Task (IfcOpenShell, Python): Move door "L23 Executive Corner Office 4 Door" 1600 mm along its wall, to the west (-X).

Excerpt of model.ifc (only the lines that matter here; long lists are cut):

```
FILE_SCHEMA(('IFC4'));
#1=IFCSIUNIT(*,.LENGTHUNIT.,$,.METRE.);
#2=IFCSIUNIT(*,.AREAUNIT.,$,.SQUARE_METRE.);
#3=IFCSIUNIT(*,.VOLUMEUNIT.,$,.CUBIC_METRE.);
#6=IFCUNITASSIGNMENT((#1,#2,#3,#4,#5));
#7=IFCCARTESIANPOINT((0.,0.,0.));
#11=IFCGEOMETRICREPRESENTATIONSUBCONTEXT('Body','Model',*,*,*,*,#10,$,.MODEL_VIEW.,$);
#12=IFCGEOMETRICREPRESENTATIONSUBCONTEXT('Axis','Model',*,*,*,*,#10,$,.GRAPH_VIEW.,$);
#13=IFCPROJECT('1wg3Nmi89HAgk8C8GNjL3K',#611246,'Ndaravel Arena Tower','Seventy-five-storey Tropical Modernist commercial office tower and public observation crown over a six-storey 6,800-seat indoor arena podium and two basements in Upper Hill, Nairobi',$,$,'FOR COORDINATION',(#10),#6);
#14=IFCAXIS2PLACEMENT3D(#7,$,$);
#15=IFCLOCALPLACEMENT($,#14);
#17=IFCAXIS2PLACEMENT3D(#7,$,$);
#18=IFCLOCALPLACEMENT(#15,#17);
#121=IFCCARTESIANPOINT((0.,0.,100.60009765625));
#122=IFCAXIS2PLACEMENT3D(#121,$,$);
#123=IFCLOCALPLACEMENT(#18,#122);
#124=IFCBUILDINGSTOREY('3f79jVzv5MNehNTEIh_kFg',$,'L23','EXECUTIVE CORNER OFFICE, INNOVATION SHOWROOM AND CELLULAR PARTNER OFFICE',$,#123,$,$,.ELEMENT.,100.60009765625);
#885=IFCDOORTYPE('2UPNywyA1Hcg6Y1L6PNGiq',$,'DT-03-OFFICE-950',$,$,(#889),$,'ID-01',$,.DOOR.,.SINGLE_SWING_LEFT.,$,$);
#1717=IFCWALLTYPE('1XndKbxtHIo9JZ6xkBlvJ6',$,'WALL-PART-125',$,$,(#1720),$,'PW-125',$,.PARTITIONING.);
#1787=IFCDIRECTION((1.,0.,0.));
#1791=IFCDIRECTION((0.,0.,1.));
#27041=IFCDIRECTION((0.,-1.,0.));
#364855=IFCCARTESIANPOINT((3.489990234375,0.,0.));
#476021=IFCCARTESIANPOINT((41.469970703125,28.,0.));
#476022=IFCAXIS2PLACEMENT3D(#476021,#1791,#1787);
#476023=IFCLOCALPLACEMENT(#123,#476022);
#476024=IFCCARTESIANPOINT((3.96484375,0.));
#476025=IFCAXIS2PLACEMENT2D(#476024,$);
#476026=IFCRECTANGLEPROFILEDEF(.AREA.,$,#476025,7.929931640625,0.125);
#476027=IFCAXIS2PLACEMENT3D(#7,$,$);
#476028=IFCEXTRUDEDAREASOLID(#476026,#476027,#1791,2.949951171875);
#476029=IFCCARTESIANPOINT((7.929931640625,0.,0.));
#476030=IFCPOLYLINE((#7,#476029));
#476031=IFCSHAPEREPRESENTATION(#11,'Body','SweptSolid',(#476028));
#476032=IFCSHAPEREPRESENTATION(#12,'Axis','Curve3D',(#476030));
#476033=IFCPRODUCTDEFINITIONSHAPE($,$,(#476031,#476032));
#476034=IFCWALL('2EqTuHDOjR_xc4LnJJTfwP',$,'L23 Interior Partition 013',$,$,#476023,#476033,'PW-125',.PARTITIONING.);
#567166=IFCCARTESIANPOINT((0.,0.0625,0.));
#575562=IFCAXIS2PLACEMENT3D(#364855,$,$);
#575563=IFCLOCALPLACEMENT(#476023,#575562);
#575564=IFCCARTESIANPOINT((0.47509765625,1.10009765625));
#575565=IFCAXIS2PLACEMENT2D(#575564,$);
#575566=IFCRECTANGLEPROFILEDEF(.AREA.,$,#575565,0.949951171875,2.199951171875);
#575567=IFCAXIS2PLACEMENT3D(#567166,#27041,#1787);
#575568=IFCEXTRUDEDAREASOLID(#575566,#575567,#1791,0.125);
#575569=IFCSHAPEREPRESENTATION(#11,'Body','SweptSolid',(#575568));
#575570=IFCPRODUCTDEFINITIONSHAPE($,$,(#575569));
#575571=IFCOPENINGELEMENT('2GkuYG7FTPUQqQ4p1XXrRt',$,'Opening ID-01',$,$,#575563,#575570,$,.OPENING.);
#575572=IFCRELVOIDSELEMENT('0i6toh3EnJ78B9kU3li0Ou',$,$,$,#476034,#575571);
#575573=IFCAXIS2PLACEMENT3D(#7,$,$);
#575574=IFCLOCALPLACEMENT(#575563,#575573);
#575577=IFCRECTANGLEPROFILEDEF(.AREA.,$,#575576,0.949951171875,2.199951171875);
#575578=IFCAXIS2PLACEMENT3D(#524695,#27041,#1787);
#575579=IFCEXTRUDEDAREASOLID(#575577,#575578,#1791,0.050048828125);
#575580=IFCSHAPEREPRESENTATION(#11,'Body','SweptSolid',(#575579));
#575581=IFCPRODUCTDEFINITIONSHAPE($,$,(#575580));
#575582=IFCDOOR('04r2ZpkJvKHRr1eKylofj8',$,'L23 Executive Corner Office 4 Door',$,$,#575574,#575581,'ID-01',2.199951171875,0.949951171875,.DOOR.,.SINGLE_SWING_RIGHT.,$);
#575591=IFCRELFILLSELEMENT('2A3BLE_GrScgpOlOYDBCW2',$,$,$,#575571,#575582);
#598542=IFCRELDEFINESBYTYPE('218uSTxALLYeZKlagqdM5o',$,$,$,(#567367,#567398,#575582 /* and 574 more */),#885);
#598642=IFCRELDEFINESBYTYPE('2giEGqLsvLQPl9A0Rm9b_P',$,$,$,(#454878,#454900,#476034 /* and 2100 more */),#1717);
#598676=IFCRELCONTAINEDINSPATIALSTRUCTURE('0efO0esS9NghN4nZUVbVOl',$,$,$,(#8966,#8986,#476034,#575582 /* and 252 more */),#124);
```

```python
import ifcopenshell
import ifcopenshell.api.geometry
import ifcopenshell.util.placement

model = ifcopenshell.open("model.ifc")

door = model.by_id(575582)
opening = door.FillsVoids[0].RelatingOpeningElement
wall = opening.VoidsElements[0].RelatingBuildingElement

wall_matrix = ifcopenshell.util.placement.get_local_placement(wall.ObjectPlacement)
shift = wall_matrix[:3, 0] * -1.6
before = ifcopenshell.util.placement.get_local_placement(door.ObjectPlacement)[:3, 3].copy()

# The door is placed relative to its opening, so it follows when the opening moves.
matrix = ifcopenshell.util.placement.get_local_placement(opening.ObjectPlacement)
matrix[:3, 3] += shift
ifcopenshell.api.geometry.edit_object_placement(
    model, product=opening, matrix=matrix, is_si=False, should_transform_children=True
)

after = ifcopenshell.util.placement.get_local_placement(door.ObjectPlacement)[:3, 3]
print("door moved by", (after - before).round(3) + 0.0)

model.write("model_v2.ifc")
```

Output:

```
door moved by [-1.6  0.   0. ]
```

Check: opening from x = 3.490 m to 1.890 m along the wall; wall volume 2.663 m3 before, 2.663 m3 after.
